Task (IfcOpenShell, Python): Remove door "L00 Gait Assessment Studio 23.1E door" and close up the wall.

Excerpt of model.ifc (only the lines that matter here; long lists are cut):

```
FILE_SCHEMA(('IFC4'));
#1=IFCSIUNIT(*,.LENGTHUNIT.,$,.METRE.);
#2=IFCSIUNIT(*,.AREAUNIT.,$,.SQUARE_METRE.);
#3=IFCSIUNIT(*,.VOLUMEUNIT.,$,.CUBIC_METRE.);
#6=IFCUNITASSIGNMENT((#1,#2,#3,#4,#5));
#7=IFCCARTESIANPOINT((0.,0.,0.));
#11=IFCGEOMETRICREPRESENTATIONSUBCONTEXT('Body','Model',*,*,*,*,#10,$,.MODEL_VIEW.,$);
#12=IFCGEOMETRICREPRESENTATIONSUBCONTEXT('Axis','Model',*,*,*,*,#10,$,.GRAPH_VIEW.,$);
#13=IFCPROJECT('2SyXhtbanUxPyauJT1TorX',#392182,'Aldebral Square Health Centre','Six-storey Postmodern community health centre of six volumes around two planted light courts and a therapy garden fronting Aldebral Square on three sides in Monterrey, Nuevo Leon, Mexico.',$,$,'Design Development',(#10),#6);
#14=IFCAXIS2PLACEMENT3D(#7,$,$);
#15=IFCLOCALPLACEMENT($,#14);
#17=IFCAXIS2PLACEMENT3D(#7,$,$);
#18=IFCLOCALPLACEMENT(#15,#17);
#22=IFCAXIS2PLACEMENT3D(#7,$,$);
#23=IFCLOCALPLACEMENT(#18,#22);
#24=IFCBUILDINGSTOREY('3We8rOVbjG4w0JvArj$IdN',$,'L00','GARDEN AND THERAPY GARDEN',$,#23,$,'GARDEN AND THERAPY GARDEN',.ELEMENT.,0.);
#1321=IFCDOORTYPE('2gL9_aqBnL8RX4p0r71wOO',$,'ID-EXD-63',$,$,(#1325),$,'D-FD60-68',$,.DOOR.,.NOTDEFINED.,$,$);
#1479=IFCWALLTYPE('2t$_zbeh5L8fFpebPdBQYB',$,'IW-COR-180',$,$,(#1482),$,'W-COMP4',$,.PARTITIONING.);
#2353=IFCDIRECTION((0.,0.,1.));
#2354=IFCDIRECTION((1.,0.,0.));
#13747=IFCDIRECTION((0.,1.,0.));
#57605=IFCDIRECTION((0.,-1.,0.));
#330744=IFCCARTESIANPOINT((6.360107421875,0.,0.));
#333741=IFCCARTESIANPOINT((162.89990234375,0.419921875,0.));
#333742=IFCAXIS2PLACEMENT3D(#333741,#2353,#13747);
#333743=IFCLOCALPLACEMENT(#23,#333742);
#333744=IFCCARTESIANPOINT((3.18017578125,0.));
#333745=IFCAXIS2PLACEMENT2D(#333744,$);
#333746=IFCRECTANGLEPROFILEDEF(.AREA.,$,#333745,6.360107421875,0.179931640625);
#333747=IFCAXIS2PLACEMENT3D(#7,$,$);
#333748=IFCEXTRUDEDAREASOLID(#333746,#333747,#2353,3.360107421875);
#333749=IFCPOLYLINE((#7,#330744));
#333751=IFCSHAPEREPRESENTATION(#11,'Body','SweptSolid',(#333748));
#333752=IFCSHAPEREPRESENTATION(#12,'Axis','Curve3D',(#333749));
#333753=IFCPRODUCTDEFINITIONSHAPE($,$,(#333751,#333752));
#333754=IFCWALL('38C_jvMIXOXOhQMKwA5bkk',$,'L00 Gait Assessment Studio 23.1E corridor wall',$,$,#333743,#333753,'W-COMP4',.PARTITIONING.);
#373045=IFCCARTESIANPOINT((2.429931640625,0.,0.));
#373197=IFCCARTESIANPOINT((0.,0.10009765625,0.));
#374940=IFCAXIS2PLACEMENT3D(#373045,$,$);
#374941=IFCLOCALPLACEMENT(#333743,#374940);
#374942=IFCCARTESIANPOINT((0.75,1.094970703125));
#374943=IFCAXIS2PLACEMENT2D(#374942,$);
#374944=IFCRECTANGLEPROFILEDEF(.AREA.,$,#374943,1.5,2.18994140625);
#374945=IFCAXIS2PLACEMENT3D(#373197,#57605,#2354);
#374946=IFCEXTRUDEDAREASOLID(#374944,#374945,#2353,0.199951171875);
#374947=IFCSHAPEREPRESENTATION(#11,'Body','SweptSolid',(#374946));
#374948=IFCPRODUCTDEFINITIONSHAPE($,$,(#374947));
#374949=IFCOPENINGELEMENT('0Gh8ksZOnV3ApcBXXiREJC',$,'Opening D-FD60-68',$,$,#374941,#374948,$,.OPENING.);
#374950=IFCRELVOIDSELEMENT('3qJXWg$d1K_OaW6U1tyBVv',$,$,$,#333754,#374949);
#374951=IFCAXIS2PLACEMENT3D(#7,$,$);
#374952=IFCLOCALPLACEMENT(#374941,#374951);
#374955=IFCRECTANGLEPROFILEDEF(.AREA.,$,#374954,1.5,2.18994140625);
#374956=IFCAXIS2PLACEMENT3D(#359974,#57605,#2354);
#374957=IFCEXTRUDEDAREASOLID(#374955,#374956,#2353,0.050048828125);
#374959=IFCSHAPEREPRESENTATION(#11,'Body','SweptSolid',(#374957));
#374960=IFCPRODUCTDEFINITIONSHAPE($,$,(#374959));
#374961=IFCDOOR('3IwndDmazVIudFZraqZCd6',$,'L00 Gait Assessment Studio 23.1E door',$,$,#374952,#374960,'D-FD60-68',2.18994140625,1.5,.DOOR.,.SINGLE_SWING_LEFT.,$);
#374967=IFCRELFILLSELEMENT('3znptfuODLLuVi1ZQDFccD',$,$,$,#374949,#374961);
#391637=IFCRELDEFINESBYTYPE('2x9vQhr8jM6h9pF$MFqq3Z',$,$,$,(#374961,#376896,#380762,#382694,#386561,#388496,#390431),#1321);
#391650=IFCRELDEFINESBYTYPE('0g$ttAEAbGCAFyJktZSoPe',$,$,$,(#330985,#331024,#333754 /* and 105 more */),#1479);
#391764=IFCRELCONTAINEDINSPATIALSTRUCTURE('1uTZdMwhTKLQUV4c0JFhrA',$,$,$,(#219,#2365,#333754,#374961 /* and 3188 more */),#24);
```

```python
import ifcopenshell
import ifcopenshell.api.feature
import ifcopenshell.api.root
import ifcopenshell.geom
import ifcopenshell.util.shape

model = ifcopenshell.open("model.ifc")
settings = ifcopenshell.geom.settings()


def volume(element):
    """Net volume in cubic metres, openings subtracted."""
    shape = ifcopenshell.geom.create_shape(settings, element)
    return ifcopenshell.util.shape.get_volume(shape.geometry)


door = model.by_guid("3IwndDmazVIudFZraqZCd6")
opening = door.FillsVoids[0].RelatingOpeningElement
wall = opening.VoidsElements[0].RelatingBuildingElement
before = volume(wall)

ifcopenshell.api.root.remove_product(model, product=door)
ifcopenshell.api.feature.remove_feature(model, feature=opening)

after = volume(wall)

print(f"wall volume {before:.3f} -> {after:.3f} m3")

model.write("model_edited.ifc")
```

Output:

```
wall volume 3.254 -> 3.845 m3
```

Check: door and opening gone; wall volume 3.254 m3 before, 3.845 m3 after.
